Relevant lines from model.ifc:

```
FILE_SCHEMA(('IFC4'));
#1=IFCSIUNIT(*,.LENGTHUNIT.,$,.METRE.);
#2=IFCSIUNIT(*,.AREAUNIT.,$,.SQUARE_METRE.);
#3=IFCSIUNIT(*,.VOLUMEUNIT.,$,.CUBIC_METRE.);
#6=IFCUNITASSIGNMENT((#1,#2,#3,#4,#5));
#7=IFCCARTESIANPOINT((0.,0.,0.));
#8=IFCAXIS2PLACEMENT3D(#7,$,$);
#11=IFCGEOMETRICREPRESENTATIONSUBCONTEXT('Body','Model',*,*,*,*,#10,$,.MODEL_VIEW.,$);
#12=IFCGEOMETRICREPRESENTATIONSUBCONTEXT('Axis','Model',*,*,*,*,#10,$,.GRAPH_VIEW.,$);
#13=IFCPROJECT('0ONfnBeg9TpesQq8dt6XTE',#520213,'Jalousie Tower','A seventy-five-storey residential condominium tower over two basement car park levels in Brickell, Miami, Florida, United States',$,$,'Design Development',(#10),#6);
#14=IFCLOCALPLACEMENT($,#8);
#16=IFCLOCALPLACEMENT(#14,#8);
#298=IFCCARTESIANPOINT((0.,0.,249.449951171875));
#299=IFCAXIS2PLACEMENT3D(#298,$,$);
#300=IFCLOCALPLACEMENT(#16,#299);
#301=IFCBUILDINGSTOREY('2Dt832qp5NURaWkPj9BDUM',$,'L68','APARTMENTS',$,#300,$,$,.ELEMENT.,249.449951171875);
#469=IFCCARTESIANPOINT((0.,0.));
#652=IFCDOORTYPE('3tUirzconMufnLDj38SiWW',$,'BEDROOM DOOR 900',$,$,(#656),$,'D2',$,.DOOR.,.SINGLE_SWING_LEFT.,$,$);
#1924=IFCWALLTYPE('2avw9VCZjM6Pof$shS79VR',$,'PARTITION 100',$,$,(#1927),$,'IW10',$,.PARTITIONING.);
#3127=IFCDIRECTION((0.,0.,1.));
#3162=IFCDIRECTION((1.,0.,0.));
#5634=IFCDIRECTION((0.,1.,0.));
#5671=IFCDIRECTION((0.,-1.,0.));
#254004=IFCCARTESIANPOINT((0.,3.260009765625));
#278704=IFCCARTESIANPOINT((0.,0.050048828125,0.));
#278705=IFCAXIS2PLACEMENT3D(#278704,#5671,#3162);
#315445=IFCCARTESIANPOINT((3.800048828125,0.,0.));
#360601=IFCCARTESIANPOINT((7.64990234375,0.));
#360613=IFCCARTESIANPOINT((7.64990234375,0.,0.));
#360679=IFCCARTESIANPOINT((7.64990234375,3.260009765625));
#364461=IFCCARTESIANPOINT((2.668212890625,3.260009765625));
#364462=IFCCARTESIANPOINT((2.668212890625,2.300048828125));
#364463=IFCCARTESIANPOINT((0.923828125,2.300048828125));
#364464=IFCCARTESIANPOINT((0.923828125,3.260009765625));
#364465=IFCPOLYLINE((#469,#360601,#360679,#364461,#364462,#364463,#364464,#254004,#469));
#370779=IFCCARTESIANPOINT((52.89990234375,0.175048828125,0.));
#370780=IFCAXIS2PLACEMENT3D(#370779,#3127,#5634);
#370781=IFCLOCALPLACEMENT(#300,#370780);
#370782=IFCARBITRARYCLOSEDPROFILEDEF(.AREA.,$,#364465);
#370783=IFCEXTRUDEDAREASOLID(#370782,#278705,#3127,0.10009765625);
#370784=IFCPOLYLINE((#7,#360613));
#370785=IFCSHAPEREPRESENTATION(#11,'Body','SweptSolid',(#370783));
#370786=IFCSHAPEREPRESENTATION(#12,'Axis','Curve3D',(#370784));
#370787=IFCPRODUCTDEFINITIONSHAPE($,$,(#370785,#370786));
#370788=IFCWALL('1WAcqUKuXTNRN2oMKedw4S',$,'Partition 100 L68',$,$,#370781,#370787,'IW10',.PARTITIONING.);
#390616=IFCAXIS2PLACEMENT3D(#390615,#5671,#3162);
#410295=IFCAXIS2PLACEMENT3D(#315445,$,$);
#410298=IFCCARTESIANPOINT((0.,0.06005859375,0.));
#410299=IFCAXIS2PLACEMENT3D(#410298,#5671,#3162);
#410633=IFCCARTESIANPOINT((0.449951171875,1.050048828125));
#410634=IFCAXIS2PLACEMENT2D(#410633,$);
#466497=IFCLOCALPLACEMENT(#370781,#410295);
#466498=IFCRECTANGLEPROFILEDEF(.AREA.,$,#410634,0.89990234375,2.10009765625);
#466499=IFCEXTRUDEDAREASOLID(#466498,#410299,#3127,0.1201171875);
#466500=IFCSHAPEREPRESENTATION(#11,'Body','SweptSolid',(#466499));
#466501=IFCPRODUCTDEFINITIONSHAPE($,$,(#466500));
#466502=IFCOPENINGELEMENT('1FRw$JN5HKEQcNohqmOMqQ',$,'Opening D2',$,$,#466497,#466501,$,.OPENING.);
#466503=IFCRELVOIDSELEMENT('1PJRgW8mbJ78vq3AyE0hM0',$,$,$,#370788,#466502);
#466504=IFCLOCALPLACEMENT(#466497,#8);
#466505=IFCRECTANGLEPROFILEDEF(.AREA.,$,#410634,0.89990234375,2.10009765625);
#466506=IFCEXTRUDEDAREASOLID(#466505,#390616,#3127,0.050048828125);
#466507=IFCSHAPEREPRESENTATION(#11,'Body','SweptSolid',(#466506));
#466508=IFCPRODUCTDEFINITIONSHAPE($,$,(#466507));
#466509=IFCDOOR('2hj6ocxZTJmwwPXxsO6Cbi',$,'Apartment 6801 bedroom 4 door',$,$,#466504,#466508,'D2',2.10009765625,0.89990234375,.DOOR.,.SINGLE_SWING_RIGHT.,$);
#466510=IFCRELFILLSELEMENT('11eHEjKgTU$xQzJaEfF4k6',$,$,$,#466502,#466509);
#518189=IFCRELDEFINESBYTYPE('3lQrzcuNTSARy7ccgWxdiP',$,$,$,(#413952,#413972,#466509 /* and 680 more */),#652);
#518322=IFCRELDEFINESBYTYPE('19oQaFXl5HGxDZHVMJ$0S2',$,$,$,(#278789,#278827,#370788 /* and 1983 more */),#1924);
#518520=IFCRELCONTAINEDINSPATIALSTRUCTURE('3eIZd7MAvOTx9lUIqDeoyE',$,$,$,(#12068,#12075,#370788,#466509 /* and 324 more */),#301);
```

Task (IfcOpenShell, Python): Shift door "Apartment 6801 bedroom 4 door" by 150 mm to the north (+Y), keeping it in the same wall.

```python
import ifcopenshell
import ifcopenshell.api.geometry
import ifcopenshell.util.placement
import ifcopenshell.util.unit

model = ifcopenshell.open("model.ifc")
unit_scale = ifcopenshell.util.unit.calculate_unit_scale(model)

door = model.by_guid("2hj6ocxZTJmwwPXxsO6Cbi")
opening = door.FillsVoids[0].RelatingOpeningElement
wall = opening.VoidsElements[0].RelatingBuildingElement

wall_matrix = ifcopenshell.util.placement.get_local_placement(wall.ObjectPlacement)
shift = wall_matrix[:3, 0] * 0.15 / unit_scale
before = ifcopenshell.util.placement.get_local_placement(door.ObjectPlacement)[:3, 3].copy()

# The door is placed relative to its opening, so it follows when the opening moves.
matrix = ifcopenshell.util.placement.get_local_placement(opening.ObjectPlacement)
matrix[:3, 3] += shift
ifcopenshell.api.geometry.edit_object_placement(
    model, product=opening, matrix=matrix, is_si=False, should_transform_children=True
)

after = ifcopenshell.util.placement.get_local_placement(door.ObjectPlacement)[:3, 3]
print("door moved by", (after - before).round(3) + 0.0)

model.write("model-out.ifc")
```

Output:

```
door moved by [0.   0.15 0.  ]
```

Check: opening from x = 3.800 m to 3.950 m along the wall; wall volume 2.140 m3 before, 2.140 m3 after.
